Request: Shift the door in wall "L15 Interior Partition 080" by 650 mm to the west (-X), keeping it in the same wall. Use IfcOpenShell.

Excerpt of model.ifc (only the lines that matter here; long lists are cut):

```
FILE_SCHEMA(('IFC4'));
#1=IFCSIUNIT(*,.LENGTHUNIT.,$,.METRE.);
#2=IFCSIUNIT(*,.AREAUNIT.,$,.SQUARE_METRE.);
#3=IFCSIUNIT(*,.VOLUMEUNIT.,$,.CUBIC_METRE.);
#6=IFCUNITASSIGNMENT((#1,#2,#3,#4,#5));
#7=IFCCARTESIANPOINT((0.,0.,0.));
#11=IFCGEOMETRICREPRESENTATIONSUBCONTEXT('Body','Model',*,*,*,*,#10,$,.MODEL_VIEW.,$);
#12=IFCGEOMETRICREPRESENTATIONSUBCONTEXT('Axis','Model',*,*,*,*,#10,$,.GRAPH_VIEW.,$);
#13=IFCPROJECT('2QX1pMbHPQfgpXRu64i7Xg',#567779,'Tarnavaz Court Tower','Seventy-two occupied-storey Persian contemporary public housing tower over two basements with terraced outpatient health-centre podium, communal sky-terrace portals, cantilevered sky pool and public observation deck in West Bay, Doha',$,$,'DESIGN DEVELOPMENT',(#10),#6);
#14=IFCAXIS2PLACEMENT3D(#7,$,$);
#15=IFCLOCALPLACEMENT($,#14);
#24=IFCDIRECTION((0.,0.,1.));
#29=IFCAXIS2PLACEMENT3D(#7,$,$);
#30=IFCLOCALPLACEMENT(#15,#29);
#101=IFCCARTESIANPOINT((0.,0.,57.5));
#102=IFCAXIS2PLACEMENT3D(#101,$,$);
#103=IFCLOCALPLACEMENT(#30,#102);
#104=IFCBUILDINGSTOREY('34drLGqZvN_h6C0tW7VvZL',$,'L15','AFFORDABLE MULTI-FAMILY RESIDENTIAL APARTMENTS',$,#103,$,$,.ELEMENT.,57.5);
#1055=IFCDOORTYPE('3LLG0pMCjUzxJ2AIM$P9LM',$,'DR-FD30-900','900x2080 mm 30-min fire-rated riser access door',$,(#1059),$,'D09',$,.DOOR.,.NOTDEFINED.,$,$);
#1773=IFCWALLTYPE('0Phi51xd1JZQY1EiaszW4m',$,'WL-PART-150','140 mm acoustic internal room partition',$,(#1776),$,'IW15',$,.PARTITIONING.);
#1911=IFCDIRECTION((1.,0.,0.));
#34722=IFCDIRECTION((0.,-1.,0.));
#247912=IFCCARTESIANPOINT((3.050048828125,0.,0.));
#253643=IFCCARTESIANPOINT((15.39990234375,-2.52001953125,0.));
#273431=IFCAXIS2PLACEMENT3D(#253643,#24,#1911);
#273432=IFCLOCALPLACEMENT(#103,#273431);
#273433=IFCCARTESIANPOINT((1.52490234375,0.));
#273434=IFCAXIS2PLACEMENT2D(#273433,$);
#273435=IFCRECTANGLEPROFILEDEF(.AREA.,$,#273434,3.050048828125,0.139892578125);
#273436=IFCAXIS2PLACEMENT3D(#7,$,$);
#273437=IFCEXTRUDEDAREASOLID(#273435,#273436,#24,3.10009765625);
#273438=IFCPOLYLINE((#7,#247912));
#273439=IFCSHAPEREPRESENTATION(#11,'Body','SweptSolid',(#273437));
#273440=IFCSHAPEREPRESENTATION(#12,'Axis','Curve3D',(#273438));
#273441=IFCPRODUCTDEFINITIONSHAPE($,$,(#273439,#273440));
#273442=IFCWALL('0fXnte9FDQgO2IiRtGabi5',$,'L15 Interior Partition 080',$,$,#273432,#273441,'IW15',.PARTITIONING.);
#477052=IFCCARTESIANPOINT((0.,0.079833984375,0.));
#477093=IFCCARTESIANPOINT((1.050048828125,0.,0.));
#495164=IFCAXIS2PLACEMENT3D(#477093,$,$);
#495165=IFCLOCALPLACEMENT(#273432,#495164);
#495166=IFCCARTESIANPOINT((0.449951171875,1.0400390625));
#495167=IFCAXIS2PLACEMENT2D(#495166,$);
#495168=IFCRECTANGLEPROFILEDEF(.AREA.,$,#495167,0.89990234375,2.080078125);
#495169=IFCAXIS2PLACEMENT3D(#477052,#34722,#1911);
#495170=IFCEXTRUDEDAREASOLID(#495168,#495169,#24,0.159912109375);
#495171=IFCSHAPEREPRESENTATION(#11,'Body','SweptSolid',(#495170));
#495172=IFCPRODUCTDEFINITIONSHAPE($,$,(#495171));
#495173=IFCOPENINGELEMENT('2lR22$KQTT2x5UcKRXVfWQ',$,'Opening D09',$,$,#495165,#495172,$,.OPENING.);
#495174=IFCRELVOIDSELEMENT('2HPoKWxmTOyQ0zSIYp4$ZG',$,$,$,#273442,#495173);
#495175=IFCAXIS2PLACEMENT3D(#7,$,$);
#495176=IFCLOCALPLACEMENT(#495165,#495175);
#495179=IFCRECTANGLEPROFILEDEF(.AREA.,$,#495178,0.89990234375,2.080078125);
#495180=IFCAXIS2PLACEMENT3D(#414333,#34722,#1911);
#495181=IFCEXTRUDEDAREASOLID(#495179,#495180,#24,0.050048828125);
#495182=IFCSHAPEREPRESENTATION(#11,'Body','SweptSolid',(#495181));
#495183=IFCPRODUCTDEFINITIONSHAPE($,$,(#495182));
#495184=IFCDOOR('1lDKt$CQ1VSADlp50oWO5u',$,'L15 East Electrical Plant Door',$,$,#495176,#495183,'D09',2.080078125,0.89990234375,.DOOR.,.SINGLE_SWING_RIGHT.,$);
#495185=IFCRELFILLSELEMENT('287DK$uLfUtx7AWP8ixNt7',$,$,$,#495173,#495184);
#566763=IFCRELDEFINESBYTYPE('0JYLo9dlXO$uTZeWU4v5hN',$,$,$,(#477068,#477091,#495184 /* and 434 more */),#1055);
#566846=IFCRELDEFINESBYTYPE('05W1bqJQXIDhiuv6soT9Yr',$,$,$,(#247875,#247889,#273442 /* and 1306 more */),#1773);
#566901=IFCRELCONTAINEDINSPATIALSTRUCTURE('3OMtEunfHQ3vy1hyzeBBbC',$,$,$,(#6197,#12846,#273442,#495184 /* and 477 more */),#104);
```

```python
import ifcopenshell
import ifcopenshell.api.geometry
import ifcopenshell.util.placement

model = ifcopenshell.open("model.ifc")

door = model.by_guid("1lDKt$CQ1VSADlp50oWO5u")
opening = door.FillsVoids[0].RelatingOpeningElement
wall = opening.VoidsElements[0].RelatingBuildingElement

wall_matrix = ifcopenshell.util.placement.get_local_placement(wall.ObjectPlacement)
shift = wall_matrix[:3, 0] * -0.65
before = ifcopenshell.util.placement.get_local_placement(door.ObjectPlacement)[:3, 3].copy()

# The door is placed relative to its opening, so it follows when the opening moves.
matrix = ifcopenshell.util.placement.get_local_placement(opening.ObjectPlacement)
matrix[:3, 3] += shift
ifcopenshell.api.geometry.edit_object_placement(
    model, product=opening, matrix=matrix, is_si=False, should_transform_children=True
)

after = ifcopenshell.util.placement.get_local_placement(door.ObjectPlacement)[:3, 3]
print("door moved by", (after - before).round(3) + 0.0)

model.write("model_rev.ifc")
```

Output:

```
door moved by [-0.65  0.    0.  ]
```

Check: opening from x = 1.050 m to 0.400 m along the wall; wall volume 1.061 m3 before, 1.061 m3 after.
